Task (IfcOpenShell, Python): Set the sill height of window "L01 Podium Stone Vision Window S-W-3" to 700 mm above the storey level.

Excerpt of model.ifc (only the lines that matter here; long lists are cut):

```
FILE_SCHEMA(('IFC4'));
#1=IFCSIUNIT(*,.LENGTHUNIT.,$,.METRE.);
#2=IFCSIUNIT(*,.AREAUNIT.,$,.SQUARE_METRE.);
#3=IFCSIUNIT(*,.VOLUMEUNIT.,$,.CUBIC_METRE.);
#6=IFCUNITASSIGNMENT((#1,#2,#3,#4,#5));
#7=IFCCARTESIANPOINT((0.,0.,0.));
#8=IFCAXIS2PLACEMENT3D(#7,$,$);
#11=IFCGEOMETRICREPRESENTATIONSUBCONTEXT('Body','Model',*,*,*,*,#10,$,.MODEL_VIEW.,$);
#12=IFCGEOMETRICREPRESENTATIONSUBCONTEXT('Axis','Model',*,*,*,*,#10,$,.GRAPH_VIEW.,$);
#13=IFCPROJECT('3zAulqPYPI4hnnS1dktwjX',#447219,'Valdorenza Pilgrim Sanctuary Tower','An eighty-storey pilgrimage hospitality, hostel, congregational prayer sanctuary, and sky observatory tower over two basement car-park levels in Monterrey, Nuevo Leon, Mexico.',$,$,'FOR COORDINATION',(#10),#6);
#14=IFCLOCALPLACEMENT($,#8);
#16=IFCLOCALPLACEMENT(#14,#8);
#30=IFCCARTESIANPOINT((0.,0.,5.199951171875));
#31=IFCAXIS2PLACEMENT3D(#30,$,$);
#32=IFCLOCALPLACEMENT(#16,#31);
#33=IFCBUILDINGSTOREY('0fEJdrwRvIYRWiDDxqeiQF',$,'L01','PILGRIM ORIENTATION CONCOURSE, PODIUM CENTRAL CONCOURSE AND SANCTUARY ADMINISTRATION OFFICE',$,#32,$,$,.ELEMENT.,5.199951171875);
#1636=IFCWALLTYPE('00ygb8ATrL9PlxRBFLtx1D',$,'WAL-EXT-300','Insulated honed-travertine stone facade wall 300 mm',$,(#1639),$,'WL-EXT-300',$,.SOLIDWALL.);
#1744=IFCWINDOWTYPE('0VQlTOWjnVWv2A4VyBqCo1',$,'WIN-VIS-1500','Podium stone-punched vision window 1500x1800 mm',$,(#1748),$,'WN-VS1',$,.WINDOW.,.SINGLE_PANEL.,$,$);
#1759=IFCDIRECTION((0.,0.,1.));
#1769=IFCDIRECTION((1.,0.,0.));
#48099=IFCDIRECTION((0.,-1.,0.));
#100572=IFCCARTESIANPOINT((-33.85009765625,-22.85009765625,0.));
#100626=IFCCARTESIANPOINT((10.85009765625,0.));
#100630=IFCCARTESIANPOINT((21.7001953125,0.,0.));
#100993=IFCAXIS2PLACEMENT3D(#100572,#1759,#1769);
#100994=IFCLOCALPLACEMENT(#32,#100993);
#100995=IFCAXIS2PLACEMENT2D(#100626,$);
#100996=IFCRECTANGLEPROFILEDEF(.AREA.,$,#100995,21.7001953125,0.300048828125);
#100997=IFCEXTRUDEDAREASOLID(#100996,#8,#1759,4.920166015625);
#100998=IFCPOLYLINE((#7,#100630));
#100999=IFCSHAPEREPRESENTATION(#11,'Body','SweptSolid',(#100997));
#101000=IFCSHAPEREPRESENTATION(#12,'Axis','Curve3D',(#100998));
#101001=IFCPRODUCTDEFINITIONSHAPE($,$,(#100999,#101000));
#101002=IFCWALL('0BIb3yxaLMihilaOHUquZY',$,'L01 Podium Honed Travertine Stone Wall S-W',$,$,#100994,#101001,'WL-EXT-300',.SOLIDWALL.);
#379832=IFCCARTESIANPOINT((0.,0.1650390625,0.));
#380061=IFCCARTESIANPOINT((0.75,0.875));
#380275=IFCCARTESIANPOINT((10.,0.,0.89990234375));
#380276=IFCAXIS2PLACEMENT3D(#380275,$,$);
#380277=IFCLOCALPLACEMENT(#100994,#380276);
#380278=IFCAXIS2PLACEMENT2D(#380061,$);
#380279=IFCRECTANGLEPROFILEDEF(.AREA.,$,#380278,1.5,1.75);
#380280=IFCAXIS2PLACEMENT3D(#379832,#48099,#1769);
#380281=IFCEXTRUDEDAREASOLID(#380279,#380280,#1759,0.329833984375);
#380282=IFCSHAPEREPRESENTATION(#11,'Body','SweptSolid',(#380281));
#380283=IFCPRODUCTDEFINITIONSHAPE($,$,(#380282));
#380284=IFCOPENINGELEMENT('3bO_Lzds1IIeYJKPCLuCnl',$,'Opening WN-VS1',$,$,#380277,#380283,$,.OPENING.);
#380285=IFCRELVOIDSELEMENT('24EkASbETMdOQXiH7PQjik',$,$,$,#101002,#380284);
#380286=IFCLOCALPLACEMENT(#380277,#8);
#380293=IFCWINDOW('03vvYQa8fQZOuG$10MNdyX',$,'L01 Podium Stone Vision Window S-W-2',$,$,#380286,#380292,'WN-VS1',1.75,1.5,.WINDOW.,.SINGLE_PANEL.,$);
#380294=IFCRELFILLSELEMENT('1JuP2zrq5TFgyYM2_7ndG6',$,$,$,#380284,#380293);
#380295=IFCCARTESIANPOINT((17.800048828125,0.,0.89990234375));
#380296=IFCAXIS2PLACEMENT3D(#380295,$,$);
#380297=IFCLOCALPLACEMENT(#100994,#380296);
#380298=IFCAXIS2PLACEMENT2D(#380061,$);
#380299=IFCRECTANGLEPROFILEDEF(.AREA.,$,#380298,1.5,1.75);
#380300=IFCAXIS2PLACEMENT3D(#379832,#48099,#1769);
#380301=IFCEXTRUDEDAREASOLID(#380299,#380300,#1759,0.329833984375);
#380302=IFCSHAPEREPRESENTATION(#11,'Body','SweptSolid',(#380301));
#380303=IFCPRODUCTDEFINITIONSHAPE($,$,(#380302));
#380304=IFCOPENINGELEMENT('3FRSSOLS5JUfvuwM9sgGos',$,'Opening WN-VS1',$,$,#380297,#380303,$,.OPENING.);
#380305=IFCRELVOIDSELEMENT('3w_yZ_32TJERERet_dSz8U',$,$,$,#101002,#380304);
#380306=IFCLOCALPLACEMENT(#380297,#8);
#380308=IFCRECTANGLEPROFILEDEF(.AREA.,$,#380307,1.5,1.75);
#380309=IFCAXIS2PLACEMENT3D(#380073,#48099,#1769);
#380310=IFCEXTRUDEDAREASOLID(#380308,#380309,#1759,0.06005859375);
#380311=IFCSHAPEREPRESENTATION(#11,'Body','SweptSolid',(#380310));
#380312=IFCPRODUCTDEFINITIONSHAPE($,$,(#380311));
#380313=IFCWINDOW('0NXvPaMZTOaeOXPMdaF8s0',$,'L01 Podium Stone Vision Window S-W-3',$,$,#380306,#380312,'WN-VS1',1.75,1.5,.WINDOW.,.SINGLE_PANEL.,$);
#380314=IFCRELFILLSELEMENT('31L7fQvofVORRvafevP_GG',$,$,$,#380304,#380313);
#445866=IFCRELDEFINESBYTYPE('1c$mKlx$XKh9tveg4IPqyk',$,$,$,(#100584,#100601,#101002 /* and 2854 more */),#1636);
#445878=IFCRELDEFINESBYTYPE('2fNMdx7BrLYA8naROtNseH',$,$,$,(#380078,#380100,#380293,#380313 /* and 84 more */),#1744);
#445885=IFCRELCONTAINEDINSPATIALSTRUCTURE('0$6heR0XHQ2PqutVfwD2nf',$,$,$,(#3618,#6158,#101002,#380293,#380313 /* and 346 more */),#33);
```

```python
import numpy as np
import ifcopenshell
import ifcopenshell.api.geometry
import ifcopenshell.geom
import ifcopenshell.util.element
import ifcopenshell.util.placement
import ifcopenshell.util.shape
import ifcopenshell.util.unit

model = ifcopenshell.open("model.ifc")
unit_scale = ifcopenshell.util.unit.calculate_unit_scale(model)

window = model.by_guid("0NXvPaMZTOaeOXPMdaF8s0")
opening = window.FillsVoids[0].RelatingOpeningElement
storey = ifcopenshell.util.element.get_container(window, ifc_class="IfcBuildingStorey")
level = ifcopenshell.util.placement.get_local_placement(storey.ObjectPlacement)[2, 3]

# The opening's origin need not be at the sill, so measure its lowest point.
shape = ifcopenshell.geom.create_shape(ifcopenshell.geom.settings(), opening)
bottom = ifcopenshell.util.shape.get_shape_bottom_elevation(shape, shape.geometry) / unit_scale
dz = level + 0.7 / unit_scale - bottom

shift = np.array([0.0, 0.0, dz])
# The window is placed relative to its opening, so it follows when the opening moves.
matrix = ifcopenshell.util.placement.get_local_placement(opening.ObjectPlacement)
matrix[:3, 3] += shift
ifcopenshell.api.geometry.edit_object_placement(
    model, product=opening, matrix=matrix, is_si=False, should_transform_children=True
)

print(f"moved by {dz * unit_scale:+.3f} m")

model.write("model_updated.ifc")
```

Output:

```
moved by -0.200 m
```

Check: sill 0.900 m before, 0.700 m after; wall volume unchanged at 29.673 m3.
